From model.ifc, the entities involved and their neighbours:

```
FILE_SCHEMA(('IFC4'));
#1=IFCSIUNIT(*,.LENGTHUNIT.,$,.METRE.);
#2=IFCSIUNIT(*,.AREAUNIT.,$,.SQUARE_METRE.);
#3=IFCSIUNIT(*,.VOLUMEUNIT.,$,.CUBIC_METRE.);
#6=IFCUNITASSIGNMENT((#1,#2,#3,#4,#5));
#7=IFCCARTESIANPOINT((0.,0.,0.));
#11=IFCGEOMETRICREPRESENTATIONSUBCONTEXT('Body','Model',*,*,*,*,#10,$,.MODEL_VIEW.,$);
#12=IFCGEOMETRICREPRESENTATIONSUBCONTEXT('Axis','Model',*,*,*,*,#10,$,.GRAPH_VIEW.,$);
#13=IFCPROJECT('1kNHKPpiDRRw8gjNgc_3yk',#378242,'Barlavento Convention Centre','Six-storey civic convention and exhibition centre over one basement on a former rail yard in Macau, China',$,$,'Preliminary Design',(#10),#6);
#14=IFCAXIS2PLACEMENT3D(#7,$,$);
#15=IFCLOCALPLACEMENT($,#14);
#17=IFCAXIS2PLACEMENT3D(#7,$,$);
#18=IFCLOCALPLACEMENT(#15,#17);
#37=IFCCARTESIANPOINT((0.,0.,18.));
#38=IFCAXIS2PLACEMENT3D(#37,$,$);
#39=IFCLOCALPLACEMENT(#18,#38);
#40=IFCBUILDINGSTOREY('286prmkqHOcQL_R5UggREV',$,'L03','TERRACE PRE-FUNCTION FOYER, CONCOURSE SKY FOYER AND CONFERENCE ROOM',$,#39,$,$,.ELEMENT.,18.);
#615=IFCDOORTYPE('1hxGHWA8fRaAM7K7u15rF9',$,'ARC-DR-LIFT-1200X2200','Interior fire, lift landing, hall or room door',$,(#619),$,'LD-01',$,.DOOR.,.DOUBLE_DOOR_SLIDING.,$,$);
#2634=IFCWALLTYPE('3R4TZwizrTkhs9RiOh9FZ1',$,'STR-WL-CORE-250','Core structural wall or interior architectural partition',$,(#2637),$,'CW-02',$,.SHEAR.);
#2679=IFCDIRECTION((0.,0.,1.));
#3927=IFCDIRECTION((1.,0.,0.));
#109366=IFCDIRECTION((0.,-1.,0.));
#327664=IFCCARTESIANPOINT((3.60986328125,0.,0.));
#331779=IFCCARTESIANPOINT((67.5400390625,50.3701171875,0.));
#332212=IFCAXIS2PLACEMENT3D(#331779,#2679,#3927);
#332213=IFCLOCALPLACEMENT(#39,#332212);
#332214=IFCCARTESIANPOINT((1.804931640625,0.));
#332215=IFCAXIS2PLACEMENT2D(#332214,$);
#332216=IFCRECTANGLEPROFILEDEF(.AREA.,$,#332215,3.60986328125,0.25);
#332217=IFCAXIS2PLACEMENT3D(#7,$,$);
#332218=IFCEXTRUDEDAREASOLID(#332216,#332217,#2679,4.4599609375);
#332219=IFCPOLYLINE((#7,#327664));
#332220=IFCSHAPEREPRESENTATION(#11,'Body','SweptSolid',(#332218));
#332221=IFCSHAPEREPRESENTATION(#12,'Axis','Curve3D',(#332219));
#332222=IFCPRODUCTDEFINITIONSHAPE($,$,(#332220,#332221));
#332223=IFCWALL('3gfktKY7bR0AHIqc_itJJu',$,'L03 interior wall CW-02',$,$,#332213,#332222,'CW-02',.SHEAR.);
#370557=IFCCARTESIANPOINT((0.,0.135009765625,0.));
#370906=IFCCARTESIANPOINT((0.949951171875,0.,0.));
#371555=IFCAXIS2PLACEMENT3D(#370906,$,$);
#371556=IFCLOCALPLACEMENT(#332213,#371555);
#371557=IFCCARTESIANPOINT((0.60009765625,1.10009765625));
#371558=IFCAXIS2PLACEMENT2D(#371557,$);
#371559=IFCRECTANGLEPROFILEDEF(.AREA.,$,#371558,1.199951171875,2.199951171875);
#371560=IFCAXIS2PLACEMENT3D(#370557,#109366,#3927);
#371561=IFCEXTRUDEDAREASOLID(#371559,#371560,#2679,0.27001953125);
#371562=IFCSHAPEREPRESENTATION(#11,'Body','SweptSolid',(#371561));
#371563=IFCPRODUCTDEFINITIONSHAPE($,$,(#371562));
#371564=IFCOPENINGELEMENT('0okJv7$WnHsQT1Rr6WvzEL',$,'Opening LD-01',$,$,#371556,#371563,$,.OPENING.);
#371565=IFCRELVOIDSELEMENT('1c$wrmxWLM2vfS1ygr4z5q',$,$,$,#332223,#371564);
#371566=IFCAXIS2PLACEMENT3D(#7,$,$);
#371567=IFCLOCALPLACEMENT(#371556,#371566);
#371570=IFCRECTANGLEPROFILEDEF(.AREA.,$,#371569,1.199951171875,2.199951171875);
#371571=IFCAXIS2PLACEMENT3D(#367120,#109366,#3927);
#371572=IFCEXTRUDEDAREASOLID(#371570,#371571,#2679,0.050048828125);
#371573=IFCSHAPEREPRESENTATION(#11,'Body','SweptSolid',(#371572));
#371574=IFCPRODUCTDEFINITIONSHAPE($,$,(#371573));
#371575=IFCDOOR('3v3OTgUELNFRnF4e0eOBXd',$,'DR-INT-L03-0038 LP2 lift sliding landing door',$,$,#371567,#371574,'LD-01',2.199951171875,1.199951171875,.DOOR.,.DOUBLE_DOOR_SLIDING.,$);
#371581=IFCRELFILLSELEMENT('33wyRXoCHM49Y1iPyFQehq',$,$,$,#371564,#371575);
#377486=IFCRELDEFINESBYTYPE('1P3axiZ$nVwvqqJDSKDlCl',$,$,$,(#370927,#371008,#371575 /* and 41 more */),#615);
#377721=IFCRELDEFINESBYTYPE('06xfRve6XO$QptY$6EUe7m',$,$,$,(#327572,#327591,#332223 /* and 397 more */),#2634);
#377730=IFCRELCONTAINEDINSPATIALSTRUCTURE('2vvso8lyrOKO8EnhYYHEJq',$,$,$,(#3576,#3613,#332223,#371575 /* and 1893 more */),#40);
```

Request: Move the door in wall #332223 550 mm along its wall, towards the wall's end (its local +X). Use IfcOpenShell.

```python
import ifcopenshell
import ifcopenshell.api.geometry
import ifcopenshell.util.placement
import ifcopenshell.util.unit

model = ifcopenshell.open("model.ifc")
unit_scale = ifcopenshell.util.unit.calculate_unit_scale(model)

door = model.by_guid("3v3OTgUELNFRnF4e0eOBXd")
opening = door.FillsVoids[0].RelatingOpeningElement
wall = opening.VoidsElements[0].RelatingBuildingElement

wall_matrix = ifcopenshell.util.placement.get_local_placement(wall.ObjectPlacement)
shift = wall_matrix[:3, 0] * 0.55 / unit_scale
before = ifcopenshell.util.placement.get_local_placement(door.ObjectPlacement)[:3, 3].copy()

# The door is placed relative to its opening, so it follows when the opening moves.
matrix = ifcopenshell.util.placement.get_local_placement(opening.ObjectPlacement)
matrix[:3, 3] += shift
ifcopenshell.api.geometry.edit_object_placement(
    model, product=opening, matrix=matrix, is_si=False, should_transform_children=True
)

after = ifcopenshell.util.placement.get_local_placement(door.ObjectPlacement)[:3, 3]
print("door moved by", (after - before).round(3) + 0.0)

model.write("model_updated.ifc")
```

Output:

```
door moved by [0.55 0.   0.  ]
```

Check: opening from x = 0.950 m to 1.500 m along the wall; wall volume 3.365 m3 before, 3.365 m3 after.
